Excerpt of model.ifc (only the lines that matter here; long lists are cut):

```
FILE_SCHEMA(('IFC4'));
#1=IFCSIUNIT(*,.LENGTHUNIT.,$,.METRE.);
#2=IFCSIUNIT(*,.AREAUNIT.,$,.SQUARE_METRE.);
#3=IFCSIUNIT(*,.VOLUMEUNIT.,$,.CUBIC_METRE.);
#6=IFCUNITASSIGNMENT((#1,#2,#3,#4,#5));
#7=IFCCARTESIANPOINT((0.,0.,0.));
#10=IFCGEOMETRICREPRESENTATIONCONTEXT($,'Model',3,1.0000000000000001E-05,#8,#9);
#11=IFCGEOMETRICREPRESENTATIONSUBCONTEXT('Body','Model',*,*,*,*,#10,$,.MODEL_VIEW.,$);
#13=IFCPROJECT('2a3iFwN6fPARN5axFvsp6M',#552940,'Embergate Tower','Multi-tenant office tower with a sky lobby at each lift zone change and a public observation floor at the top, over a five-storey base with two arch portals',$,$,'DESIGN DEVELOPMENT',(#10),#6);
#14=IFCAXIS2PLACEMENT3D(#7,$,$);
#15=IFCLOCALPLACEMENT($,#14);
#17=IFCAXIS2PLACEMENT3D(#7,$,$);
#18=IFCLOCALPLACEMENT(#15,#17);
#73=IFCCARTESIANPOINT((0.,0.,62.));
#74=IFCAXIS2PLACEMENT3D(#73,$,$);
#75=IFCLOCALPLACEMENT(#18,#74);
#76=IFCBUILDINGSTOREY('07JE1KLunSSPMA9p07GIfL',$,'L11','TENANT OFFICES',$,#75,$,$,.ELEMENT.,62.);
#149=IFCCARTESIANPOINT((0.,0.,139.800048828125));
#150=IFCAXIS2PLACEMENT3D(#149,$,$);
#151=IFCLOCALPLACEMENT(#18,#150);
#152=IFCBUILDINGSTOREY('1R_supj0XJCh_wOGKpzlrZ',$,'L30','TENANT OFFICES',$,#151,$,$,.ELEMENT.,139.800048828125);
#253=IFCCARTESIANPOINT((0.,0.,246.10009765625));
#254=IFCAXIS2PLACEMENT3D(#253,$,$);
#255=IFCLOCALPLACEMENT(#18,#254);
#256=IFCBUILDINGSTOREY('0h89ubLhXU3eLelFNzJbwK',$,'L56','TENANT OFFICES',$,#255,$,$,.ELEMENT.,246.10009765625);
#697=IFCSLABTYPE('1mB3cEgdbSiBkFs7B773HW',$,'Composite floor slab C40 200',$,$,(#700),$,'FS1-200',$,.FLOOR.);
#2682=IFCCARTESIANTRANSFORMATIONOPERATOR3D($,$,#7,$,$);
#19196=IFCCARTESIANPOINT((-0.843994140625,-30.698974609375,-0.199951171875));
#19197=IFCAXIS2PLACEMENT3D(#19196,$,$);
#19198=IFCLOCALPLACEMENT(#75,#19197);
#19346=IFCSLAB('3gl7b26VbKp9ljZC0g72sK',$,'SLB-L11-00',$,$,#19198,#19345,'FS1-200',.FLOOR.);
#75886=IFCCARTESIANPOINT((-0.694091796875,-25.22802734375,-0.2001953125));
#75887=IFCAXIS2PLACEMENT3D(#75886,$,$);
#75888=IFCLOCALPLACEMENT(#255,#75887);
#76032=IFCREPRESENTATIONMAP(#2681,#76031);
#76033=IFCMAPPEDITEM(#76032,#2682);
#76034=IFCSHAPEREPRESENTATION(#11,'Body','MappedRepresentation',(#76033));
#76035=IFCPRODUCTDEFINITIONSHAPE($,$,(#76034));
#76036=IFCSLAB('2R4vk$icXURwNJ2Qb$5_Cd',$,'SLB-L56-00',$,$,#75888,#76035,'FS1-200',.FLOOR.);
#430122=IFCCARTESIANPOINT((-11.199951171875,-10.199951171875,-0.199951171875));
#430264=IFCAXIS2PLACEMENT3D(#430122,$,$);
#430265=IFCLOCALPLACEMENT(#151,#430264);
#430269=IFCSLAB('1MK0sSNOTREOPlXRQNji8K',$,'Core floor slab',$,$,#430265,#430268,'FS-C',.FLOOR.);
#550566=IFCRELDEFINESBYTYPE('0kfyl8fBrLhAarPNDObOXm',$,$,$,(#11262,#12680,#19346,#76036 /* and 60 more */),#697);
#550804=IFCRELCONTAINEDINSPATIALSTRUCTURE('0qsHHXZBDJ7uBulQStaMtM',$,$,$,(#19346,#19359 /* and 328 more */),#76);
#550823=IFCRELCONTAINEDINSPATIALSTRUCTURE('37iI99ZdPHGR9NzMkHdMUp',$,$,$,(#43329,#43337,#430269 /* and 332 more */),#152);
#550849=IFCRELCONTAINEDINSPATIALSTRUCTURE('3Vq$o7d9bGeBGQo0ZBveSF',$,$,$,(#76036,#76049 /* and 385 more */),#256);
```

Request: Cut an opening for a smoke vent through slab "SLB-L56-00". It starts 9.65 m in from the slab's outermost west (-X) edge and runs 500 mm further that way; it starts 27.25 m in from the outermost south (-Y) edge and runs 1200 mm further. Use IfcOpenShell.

```python
import numpy as np
import ifcopenshell
import ifcopenshell.api.feature
import ifcopenshell.api.geometry
import ifcopenshell.api.root
import ifcopenshell.geom
import ifcopenshell.util.placement
import ifcopenshell.util.representation
import ifcopenshell.util.shape
import ifcopenshell.util.unit

model = ifcopenshell.open("model.ifc")
unit_scale = ifcopenshell.util.unit.calculate_unit_scale(model)
settings = ifcopenshell.geom.settings()


def volume(element):
    """Net volume in cubic metres, openings subtracted."""
    shape = ifcopenshell.geom.create_shape(settings, element)
    return ifcopenshell.util.shape.get_volume(shape.geometry)


slab = model.by_id(76036)
before = volume(slab)

# Extent in the slab's own axes, in metres. The edges named are its -X and -Y sides.
slab_shape = ifcopenshell.geom.create_shape(settings, slab)
vertices = ifcopenshell.util.shape.get_vertices(slab_shape.geometry)
x_min, y_min, bottom = vertices.min(axis=0)
top = vertices[:, 2].max()

opening = ifcopenshell.api.root.create_entity(model, ifc_class="IfcOpeningElement", name="Smoke vent opening", predefined_type="OPENING")
context = ifcopenshell.util.representation.get_context(model, "Model", "Body", "MODEL_VIEW")
width, depth = 0.5, 1.2
outline = [(0.0, 0.0), (width, 0.0), (width, depth), (0.0, depth), (0.0, 0.0)]
# Overshoot both faces by 50 mm so the cut is clean.
shape = ifcopenshell.api.geometry.add_slab_representation(
    model, context=context, depth=top - bottom + 0.1, polyline=outline
)
ifcopenshell.api.geometry.assign_representation(model, product=opening, representation=shape)

matrix = ifcopenshell.util.placement.get_local_placement(slab.ObjectPlacement)
matrix[:, 3] = matrix @ np.append(np.array([x_min + 9.65, y_min + 27.25, bottom - 0.05]) / unit_scale, 1.0)
ifcopenshell.api.geometry.edit_object_placement(model, product=opening, matrix=matrix, is_si=False)
ifcopenshell.api.feature.add_feature(model, feature=opening, element=slab)

after = volume(slab)

print(f"slab volume {before:.3f} -> {after:.3f} m3")

model.write("model_v2.ifc")
```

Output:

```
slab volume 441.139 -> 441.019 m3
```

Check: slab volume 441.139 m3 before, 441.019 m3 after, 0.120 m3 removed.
